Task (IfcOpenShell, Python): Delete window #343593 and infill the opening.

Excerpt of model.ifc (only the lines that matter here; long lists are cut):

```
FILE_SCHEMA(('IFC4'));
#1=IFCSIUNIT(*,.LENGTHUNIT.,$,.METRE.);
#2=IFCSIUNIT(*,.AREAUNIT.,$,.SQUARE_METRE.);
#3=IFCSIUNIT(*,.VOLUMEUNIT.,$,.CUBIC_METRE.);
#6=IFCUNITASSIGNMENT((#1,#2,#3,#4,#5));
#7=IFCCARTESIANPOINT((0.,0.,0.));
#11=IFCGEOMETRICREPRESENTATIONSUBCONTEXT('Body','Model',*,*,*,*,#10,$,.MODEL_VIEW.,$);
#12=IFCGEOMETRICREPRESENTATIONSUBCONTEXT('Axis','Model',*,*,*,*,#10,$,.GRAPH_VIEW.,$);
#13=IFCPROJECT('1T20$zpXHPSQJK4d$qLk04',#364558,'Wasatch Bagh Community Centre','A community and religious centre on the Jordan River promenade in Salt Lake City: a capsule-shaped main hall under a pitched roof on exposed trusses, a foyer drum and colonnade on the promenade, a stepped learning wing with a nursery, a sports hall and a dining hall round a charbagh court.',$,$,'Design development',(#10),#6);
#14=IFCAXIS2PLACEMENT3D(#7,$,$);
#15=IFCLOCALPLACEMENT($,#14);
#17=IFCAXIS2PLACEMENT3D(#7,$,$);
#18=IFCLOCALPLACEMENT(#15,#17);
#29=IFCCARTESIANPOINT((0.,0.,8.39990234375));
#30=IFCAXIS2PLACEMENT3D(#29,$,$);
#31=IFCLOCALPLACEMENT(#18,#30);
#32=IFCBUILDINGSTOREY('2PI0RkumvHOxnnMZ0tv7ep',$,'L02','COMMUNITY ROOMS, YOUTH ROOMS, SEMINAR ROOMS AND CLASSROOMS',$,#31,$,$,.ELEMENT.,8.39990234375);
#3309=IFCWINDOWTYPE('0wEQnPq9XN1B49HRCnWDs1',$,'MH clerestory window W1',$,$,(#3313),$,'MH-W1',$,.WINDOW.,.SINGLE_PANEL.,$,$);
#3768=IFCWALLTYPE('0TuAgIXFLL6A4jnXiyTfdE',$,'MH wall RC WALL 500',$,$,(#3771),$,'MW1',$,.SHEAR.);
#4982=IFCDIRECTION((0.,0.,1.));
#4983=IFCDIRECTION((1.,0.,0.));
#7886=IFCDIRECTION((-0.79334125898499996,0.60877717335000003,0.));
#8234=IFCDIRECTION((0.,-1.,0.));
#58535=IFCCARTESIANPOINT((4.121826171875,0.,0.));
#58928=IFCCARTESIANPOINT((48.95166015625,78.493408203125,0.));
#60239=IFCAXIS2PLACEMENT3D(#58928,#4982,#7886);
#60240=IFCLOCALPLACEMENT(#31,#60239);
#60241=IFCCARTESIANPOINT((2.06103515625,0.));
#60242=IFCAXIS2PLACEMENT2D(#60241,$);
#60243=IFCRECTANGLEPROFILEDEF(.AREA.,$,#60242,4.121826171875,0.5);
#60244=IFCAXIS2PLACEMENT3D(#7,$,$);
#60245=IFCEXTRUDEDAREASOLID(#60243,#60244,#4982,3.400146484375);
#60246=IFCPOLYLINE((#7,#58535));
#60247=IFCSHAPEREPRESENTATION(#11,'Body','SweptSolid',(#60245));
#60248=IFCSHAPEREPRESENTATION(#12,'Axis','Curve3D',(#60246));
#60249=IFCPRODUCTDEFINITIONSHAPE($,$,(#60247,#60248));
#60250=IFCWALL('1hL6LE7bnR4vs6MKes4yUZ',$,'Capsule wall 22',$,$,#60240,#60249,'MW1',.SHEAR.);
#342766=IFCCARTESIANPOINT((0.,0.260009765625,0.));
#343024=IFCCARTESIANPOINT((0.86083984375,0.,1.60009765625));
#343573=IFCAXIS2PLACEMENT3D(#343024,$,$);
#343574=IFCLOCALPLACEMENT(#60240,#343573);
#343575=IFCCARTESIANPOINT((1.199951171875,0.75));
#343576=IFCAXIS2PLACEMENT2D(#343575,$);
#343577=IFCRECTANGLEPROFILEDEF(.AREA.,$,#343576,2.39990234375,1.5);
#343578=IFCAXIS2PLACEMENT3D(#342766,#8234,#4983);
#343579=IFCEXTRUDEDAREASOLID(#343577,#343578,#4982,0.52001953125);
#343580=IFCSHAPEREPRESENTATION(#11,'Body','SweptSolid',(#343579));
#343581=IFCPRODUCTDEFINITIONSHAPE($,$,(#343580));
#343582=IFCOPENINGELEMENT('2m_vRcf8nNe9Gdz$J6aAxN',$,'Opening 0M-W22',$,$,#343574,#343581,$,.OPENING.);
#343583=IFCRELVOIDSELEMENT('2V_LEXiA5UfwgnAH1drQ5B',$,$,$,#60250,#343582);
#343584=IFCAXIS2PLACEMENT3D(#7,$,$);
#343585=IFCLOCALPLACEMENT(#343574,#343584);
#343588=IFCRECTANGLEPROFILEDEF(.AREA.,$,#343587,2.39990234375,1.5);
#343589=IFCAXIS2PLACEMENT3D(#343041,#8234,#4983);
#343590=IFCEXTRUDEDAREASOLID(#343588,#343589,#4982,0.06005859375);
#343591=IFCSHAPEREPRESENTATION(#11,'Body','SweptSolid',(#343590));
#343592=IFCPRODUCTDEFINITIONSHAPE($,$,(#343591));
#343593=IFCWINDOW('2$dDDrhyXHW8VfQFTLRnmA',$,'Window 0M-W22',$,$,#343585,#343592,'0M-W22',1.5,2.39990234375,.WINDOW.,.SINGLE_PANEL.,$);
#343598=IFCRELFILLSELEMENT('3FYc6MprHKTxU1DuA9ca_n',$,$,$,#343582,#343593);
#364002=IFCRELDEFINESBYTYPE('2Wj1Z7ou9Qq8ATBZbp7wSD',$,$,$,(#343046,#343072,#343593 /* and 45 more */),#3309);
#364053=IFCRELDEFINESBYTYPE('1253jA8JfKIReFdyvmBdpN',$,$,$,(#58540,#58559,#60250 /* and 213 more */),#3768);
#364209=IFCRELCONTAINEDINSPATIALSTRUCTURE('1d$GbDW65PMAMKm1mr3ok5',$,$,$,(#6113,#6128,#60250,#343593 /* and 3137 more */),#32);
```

```python
import ifcopenshell
import ifcopenshell.api.feature
import ifcopenshell.api.root
import ifcopenshell.geom
import ifcopenshell.util.shape

model = ifcopenshell.open("model.ifc")
settings = ifcopenshell.geom.settings()


def volume(element):
    """Net volume in cubic metres, openings subtracted."""
    shape = ifcopenshell.geom.create_shape(settings, element)
    return ifcopenshell.util.shape.get_volume(shape.geometry)


window = model.by_guid("2$dDDrhyXHW8VfQFTLRnmA")
opening = window.FillsVoids[0].RelatingOpeningElement
wall = opening.VoidsElements[0].RelatingBuildingElement
before = volume(wall)

ifcopenshell.api.root.remove_product(model, product=window)
ifcopenshell.api.feature.remove_feature(model, feature=opening)

after = volume(wall)

print(f"wall volume {before:.3f} -> {after:.3f} m3")

model.write("model_edited.ifc")
```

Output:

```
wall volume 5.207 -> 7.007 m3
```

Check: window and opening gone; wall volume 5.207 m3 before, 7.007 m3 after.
